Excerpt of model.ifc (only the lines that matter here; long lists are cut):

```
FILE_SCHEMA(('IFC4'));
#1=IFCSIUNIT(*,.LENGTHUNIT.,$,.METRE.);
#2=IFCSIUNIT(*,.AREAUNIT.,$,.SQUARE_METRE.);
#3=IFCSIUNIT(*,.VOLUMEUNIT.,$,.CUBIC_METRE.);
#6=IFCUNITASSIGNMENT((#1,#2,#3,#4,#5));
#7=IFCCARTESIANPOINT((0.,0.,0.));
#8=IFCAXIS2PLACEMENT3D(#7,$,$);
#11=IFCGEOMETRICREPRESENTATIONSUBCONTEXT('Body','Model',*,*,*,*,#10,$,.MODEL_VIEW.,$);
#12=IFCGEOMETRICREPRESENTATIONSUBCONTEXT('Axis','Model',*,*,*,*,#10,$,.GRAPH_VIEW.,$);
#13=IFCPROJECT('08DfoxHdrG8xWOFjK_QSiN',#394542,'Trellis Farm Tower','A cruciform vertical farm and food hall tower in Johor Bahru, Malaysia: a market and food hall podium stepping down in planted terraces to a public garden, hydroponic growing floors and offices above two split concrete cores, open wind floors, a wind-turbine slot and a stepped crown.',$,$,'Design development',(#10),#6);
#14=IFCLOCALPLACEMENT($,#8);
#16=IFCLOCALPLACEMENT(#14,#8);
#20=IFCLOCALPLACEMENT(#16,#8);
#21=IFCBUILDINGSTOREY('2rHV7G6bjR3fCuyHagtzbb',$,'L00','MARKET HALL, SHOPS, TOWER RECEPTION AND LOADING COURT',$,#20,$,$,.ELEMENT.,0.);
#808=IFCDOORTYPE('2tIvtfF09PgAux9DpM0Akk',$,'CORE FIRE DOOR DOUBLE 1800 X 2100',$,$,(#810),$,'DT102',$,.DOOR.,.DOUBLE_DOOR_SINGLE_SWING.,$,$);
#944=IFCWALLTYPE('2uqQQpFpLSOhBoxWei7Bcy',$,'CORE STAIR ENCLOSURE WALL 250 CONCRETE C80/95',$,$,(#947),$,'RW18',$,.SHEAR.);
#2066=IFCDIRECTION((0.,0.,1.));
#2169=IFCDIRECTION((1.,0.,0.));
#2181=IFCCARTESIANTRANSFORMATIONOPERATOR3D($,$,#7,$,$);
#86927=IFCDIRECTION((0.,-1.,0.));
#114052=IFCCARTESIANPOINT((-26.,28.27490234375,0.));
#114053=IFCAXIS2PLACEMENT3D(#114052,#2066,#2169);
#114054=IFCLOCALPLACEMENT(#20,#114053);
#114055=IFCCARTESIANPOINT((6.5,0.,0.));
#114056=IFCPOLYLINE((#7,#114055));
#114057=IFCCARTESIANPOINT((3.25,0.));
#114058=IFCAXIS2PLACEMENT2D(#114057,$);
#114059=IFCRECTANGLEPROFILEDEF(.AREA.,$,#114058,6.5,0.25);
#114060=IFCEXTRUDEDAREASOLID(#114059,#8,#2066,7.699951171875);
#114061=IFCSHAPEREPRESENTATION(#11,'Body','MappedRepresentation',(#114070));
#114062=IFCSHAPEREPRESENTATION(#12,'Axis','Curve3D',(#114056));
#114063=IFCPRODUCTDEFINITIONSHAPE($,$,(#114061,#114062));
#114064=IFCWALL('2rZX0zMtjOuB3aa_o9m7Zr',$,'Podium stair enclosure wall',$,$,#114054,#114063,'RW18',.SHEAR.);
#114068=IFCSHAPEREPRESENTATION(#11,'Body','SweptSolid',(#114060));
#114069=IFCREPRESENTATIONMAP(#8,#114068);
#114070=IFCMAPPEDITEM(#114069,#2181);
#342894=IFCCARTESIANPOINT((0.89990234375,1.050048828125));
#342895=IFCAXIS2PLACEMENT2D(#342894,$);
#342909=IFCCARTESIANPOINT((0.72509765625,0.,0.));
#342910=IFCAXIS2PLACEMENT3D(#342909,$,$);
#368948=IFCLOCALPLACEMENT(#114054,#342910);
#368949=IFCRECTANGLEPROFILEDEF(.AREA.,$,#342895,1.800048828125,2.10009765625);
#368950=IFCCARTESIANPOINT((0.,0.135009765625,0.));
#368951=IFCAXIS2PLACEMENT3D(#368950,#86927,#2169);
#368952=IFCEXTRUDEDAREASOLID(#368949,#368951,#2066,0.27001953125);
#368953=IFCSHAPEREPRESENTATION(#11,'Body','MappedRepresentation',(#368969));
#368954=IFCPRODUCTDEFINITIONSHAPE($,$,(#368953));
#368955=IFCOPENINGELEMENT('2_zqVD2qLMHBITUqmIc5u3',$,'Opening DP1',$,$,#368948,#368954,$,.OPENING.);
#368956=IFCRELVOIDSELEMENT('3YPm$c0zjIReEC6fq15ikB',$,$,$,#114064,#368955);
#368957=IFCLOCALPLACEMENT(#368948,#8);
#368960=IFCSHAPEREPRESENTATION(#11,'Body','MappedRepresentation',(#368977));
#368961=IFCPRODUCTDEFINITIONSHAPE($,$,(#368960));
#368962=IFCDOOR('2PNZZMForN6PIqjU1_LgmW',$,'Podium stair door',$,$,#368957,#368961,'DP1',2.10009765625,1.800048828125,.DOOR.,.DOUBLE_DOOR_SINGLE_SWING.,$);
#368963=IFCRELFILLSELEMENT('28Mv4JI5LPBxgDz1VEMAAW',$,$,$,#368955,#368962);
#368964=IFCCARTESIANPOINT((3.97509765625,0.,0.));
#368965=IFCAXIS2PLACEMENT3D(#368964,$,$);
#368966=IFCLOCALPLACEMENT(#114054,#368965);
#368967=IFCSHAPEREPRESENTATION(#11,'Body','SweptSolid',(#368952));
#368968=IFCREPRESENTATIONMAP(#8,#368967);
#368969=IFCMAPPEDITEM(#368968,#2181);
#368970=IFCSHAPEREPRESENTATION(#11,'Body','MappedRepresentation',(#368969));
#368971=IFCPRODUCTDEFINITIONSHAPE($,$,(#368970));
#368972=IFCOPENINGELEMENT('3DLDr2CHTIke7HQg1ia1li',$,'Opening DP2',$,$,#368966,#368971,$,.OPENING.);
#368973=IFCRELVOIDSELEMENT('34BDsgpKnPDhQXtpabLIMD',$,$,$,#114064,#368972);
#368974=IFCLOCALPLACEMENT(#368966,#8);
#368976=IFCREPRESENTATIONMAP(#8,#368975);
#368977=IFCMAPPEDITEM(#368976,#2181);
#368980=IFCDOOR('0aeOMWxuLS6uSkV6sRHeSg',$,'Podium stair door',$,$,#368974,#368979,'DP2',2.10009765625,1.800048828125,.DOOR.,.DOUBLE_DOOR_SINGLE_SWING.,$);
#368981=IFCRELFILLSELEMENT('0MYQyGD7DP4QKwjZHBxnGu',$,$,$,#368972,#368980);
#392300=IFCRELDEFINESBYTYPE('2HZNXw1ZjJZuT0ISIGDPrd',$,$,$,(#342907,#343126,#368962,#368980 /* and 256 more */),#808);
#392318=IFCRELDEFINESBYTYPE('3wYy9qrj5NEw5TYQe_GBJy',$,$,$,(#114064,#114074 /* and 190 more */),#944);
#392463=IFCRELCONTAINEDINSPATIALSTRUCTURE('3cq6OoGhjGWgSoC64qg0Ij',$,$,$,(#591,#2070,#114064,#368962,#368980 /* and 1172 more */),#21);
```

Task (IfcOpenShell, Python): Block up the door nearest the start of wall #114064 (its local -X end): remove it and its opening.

```python
import ifcopenshell
import ifcopenshell.api.feature
import ifcopenshell.api.root
import ifcopenshell.geom
import ifcopenshell.util.shape

model = ifcopenshell.open("model.ifc")
settings = ifcopenshell.geom.settings()


def volume(element):
    """Net volume in cubic metres, openings subtracted."""
    shape = ifcopenshell.geom.create_shape(settings, element)
    return ifcopenshell.util.shape.get_volume(shape.geometry)


door = model.by_id(368962)
opening = door.FillsVoids[0].RelatingOpeningElement
wall = opening.VoidsElements[0].RelatingBuildingElement
before = volume(wall)

ifcopenshell.api.root.remove_product(model, product=door)
ifcopenshell.api.feature.remove_feature(model, feature=opening)

after = volume(wall)

print(f"wall volume {before:.3f} -> {after:.3f} m3")

model.write("model_rev.ifc")
```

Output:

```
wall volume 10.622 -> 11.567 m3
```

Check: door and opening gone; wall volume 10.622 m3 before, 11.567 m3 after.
